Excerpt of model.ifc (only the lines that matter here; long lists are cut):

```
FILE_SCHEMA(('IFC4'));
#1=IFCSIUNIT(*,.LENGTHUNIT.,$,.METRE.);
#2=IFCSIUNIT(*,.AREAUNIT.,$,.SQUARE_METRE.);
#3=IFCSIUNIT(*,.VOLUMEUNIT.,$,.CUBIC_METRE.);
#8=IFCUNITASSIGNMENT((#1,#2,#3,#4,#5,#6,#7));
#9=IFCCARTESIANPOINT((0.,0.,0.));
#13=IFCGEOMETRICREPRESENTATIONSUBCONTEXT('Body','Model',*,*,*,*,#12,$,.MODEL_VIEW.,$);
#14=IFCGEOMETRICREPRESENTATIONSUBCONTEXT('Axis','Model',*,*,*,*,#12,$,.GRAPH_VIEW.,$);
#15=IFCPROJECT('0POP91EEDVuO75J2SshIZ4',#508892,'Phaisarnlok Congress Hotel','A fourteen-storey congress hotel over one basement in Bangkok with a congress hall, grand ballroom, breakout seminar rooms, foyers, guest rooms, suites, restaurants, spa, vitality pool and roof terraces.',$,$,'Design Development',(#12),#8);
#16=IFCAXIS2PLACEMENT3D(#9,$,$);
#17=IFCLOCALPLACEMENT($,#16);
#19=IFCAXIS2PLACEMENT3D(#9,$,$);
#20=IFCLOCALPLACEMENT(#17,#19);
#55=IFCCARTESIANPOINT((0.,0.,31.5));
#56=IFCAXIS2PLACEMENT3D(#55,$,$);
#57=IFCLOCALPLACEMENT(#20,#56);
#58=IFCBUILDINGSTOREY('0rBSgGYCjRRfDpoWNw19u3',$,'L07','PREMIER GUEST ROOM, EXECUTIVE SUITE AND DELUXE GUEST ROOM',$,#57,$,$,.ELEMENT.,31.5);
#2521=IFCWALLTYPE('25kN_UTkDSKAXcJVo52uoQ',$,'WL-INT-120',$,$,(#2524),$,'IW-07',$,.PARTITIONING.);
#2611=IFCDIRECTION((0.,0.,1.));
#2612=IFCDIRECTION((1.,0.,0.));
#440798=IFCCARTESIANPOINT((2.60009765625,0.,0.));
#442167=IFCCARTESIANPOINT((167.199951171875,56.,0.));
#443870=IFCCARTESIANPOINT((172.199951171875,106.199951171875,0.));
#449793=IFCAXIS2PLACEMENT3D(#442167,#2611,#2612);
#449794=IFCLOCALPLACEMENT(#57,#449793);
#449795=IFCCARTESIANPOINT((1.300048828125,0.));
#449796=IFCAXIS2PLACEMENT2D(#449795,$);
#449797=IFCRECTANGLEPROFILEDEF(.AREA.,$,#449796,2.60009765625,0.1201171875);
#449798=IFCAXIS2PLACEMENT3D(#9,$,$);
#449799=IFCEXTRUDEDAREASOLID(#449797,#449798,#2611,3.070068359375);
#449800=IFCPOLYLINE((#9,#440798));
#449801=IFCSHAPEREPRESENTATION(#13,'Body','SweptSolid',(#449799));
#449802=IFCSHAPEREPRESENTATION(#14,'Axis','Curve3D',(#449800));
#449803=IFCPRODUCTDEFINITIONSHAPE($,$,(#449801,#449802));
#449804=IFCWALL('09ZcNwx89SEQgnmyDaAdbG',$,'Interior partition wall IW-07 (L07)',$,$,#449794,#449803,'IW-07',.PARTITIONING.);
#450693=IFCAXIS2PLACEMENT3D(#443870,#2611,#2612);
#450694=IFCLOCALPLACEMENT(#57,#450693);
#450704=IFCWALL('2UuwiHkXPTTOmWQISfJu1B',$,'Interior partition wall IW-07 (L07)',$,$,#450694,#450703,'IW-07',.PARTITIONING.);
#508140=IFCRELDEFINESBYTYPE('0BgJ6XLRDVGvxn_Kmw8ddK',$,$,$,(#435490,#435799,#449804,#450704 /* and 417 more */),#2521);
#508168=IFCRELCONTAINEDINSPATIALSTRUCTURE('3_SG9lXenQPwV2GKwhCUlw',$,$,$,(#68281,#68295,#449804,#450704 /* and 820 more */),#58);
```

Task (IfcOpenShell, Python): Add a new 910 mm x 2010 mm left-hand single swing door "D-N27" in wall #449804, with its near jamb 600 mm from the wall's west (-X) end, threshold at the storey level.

```python
import numpy as np
import ifcopenshell
import ifcopenshell.api.feature
import ifcopenshell.api.geometry
import ifcopenshell.api.root
import ifcopenshell.api.spatial
import ifcopenshell.geom
import ifcopenshell.util.element
import ifcopenshell.util.placement
import ifcopenshell.util.representation
import ifcopenshell.util.shape
import ifcopenshell.util.unit

model = ifcopenshell.open("model.ifc")
unit_scale = ifcopenshell.util.unit.calculate_unit_scale(model)
settings = ifcopenshell.geom.settings()


def volume(element):
    """Net volume in cubic metres, openings subtracted."""
    shape = ifcopenshell.geom.create_shape(settings, element)
    return ifcopenshell.util.shape.get_volume(shape.geometry)


wall = model.by_id(449804)
storey = ifcopenshell.util.element.get_container(wall, ifc_class="IfcBuildingStorey")
context = ifcopenshell.util.representation.get_context(model, "Model", "Body", "MODEL_VIEW")
before = volume(wall)

width, height, from_end, sill = 0.91, 2.01, 0.6, 0.0  # metres

# The wall runs along its own X axis, and the end named is its -X end.
wall_shape = ifcopenshell.geom.create_shape(settings, wall)
x, y, z = ifcopenshell.util.shape.get_vertices(wall_shape.geometry).T
start = x.min() + from_end
face, thickness = float(y.min()), float(y.max() - y.min())
wall_matrix = ifcopenshell.util.placement.get_local_placement(wall.ObjectPlacement)
level = ifcopenshell.util.placement.get_local_placement(storey.ObjectPlacement)[2, 3]


def in_wall(x, y):
    """Placement at x, y metres in the wall's axes, at sill height."""
    matrix = wall_matrix.copy()
    matrix[:, 3] = wall_matrix @ np.array([x / unit_scale, y / unit_scale, 0.0, 1.0])
    matrix[2, 3] = level + sill / unit_scale
    return matrix


# Opening: a box that overshoots both wall faces by 50 mm.
opening = ifcopenshell.api.root.create_entity(model, ifc_class="IfcOpeningElement", predefined_type="OPENING")
box = ifcopenshell.api.geometry.add_wall_representation(
    model, context=context, length=width, height=height, thickness=thickness + 0.1
)
ifcopenshell.api.geometry.assign_representation(model, product=opening, representation=box)
ifcopenshell.api.geometry.edit_object_placement(model, product=opening, matrix=in_wall(start, face - 0.05), is_si=False)
ifcopenshell.api.feature.add_feature(model, feature=opening, element=wall)

door = ifcopenshell.api.root.create_entity(model, ifc_class="IfcDoor", name="D-N27", predefined_type="DOOR")
door.OverallWidth, door.OverallHeight = width / unit_scale, height / unit_scale
door.OperationType = "SINGLE_SWING_LEFT"
body = ifcopenshell.api.geometry.add_door_representation(
    model,
    context=context,
    overall_width=door.OverallWidth,
    overall_height=door.OverallHeight,
    operation_type="SINGLE_SWING_LEFT",
    lining_properties={"LiningDepth": thickness / unit_scale, "ThresholdDepth": thickness / unit_scale},
)
ifcopenshell.api.geometry.assign_representation(model, product=door, representation=body)
ifcopenshell.api.spatial.assign_container(model, products=[door], relating_structure=storey)
ifcopenshell.api.feature.add_filling(model, opening=opening, element=door)

# The lining spans the wall, so the door starts at the wall face.
ifcopenshell.api.geometry.edit_object_placement(model, product=door, matrix=in_wall(start, face), is_si=False)

after = volume(wall)

print(f"wall volume {before:.3f} -> {after:.3f} m3")

model.write("model_rev.ifc")
```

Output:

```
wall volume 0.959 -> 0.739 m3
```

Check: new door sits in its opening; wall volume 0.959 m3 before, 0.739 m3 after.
